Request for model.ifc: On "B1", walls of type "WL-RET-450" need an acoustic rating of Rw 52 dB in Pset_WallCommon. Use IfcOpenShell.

First a look at what the model holds.

```python
import ifcopenshell
import ifcopenshell.util.element

model = ifcopenshell.open("model.ifc")
print(model.schema)
storey = next(s for s in model.by_type("IfcBuildingStorey") if s.Name == "B1")
walls = [e for e in ifcopenshell.util.element.get_decomposition(storey) if e.is_a("IfcWall")]
seen = {}
for e in walls:
    element_type = ifcopenshell.util.element.get_type(e)
    key = (element_type.Name if element_type != e and element_type else None, ifcopenshell.util.element.get_pset(e, "Pset_WallCommon", "AcousticRating"))
    seen[key] = seen.get(key, 0) + 1
for (name, value), count in sorted(seen.items(), key=str):
    print(count, "x", name, "|", value)
```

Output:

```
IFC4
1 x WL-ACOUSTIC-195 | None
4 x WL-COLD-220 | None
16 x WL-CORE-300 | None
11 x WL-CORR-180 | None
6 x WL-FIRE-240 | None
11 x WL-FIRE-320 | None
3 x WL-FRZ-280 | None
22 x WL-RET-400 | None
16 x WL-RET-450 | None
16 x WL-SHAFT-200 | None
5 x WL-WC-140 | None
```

```python
import ifcopenshell
import ifcopenshell.api.pset
import ifcopenshell.util.element

model = ifcopenshell.open("model.ifc")

storey = next(s for s in model.by_type("IfcBuildingStorey") if s.Name == "B1")
walls = [e for e in ifcopenshell.util.element.get_decomposition(storey) if e.is_a("IfcWall")]

count = 0
for e in walls:
    element_type = ifcopenshell.util.element.get_type(e)
    if element_type in (None, e) or element_type.Name != "WL-RET-450":
        continue
    # add_pset returns the element's existing set when there is one.
    pset = ifcopenshell.api.pset.add_pset(model, product=e, name="Pset_WallCommon")
    ifcopenshell.api.pset.edit_pset(model, pset=pset, properties={"AcousticRating": "Rw 52 dB"})
    count += 1

print(count, "walls updated")

model.write("model_rev.ifc")
```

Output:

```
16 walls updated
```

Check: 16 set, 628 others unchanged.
